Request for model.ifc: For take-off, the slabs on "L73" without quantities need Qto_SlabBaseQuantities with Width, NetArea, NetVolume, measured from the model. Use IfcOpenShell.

First a look at what the model holds.

```python
import ifcopenshell
import ifcopenshell.util.element
import ifcopenshell.util.unit

model = ifcopenshell.open("model.ifc")
print(model.schema)
for unit_type in ("LENGTHUNIT", "AREAUNIT", "VOLUMEUNIT"):
    print(unit_type, ifcopenshell.util.unit.calculate_unit_scale(model, unit_type))
storey = next(s for s in model.by_type("IfcBuildingStorey") if s.Name == "L73")
slabs = [e for e in ifcopenshell.util.element.get_decomposition(storey) if e.is_a("IfcSlab")]
for e in sorted(slabs, key=lambda e: e.id()):
    print(e.id(), e.is_a(), e.Name, list(ifcopenshell.util.element.get_psets(e, qtos_only=True)), sep=" | ")
```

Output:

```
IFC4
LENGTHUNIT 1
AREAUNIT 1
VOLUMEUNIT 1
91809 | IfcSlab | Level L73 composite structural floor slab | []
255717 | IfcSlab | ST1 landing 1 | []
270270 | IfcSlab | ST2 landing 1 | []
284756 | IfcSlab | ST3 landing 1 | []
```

```python
import ifcopenshell
import ifcopenshell.api.pset
import ifcopenshell.geom
import ifcopenshell.util.element
import ifcopenshell.util.shape
import ifcopenshell.util.unit

model = ifcopenshell.open("model.ifc")
unit_scale = ifcopenshell.util.unit.calculate_unit_scale(model)
area_scale = ifcopenshell.util.unit.calculate_unit_scale(model, "AREAUNIT")
volume_scale = ifcopenshell.util.unit.calculate_unit_scale(model, "VOLUMEUNIT")
settings = ifcopenshell.geom.settings()

storey = next(s for s in model.by_type("IfcBuildingStorey") if s.Name == "L73")
slabs = [e for e in ifcopenshell.util.element.get_decomposition(storey) if e.is_a("IfcSlab")]

for e in sorted(slabs, key=lambda e: e.id()):
    if ifcopenshell.util.element.get_psets(e, qtos_only=True, should_inherit=False):
        continue
    # Geometry comes back in metres, in the element's own axes.
    shape = ifcopenshell.geom.create_shape(settings, e)
    values = {
        "Width": ifcopenshell.util.shape.get_z(shape.geometry) / unit_scale,
        "NetArea": ifcopenshell.util.shape.get_footprint_area(shape.geometry) / area_scale,
        "NetVolume": ifcopenshell.util.shape.get_volume(shape.geometry) / volume_scale,
    }
    qto = ifcopenshell.api.pset.add_qto(model, product=e, name="Qto_SlabBaseQuantities")
    ifcopenshell.api.pset.edit_qto(model, qto=qto, properties=values)
    print(e.id(), {k: round(v, 3) for k, v in values.items()})

model.write("model_rev.ifc")
```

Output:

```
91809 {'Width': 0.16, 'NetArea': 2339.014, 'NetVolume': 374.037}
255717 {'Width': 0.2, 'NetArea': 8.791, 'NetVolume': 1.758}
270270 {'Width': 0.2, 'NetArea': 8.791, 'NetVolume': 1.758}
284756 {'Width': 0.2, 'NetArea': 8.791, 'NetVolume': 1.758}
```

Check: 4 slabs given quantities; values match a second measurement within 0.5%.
